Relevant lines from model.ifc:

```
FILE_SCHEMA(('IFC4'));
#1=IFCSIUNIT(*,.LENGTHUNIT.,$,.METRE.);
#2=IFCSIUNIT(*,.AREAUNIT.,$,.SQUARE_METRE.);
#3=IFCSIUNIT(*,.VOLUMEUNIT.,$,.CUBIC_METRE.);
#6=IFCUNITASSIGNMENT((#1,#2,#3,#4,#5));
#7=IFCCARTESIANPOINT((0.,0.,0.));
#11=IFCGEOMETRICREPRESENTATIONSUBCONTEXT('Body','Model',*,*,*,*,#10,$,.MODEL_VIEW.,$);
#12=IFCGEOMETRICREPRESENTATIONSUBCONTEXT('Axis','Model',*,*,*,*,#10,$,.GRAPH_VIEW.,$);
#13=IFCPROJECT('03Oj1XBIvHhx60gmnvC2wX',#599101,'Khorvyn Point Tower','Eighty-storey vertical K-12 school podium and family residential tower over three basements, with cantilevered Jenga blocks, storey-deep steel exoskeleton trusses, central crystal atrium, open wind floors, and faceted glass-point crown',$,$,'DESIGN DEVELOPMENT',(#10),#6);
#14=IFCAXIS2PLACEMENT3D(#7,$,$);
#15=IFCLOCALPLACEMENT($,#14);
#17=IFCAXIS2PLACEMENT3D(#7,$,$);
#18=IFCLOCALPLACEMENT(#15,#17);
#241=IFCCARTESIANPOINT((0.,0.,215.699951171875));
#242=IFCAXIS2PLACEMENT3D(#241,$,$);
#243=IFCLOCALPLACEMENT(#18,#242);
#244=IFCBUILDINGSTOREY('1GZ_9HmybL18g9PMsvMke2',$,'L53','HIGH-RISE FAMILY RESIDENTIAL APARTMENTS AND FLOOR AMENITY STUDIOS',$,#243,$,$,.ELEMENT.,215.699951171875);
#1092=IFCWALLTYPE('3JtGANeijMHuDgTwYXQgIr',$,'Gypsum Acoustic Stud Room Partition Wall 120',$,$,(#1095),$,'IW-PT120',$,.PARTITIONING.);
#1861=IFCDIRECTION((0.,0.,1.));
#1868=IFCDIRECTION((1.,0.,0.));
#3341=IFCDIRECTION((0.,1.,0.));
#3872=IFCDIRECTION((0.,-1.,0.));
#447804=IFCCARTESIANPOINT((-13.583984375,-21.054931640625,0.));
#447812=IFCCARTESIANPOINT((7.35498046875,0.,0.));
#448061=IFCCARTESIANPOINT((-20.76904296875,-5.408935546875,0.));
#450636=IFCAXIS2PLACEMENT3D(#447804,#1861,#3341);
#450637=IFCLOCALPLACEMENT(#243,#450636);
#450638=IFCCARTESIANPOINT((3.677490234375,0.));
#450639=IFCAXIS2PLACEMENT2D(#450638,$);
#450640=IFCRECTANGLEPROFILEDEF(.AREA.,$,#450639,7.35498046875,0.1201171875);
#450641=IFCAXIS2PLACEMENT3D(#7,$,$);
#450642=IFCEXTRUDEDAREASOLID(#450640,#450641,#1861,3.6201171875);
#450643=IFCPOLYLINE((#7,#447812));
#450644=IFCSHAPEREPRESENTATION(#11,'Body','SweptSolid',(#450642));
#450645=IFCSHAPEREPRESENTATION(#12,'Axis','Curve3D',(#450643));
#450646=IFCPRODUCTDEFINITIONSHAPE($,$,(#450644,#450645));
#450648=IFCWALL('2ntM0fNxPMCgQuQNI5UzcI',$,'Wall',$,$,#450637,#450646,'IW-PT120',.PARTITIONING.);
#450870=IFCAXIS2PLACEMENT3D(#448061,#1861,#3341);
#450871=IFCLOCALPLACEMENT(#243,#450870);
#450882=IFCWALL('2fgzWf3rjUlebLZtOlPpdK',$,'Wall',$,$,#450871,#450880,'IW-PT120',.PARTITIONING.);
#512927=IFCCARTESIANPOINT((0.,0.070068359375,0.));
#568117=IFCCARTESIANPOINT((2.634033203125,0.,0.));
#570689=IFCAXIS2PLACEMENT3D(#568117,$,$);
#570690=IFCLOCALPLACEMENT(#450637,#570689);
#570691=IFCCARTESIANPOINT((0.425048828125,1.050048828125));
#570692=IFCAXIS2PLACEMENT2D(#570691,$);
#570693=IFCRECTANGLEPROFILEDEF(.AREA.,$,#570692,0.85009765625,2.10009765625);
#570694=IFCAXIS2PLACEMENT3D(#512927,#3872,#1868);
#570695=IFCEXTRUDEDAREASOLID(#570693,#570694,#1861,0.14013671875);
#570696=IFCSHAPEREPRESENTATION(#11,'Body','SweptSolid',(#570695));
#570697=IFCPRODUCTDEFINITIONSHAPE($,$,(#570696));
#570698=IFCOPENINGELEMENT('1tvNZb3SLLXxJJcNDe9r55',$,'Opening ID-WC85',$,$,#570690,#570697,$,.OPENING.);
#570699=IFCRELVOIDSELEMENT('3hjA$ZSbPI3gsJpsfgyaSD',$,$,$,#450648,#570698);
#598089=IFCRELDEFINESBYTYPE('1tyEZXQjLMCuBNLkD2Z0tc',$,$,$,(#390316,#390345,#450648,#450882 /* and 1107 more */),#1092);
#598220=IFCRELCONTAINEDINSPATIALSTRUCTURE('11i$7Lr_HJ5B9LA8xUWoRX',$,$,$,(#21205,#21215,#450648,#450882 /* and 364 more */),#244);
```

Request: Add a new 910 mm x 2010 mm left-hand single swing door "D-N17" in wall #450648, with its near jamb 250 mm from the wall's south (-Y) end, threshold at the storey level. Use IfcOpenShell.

```python
import numpy as np
import ifcopenshell
import ifcopenshell.api.feature
import ifcopenshell.api.geometry
import ifcopenshell.api.root
import ifcopenshell.api.spatial
import ifcopenshell.geom
import ifcopenshell.util.element
import ifcopenshell.util.placement
import ifcopenshell.util.representation
import ifcopenshell.util.shape
import ifcopenshell.util.unit

model = ifcopenshell.open("model.ifc")
unit_scale = ifcopenshell.util.unit.calculate_unit_scale(model)
settings = ifcopenshell.geom.settings()


def volume(element):
    """Net volume in cubic metres, openings subtracted."""
    shape = ifcopenshell.geom.create_shape(settings, element)
    return ifcopenshell.util.shape.get_volume(shape.geometry)


wall = model.by_guid("2ntM0fNxPMCgQuQNI5UzcI")
storey = ifcopenshell.util.element.get_container(wall, ifc_class="IfcBuildingStorey")
context = ifcopenshell.util.representation.get_context(model, "Model", "Body", "MODEL_VIEW")
before = volume(wall)

width, height, from_end, sill = 0.91, 2.01, 0.25, 0.0  # metres

# The wall runs along its own X axis, and the end named is its -X end.
wall_shape = ifcopenshell.geom.create_shape(settings, wall)
x, y, z = ifcopenshell.util.shape.get_vertices(wall_shape.geometry).T
start = x.min() + from_end
face, thickness = float(y.min()), float(y.max() - y.min())
wall_matrix = ifcopenshell.util.placement.get_local_placement(wall.ObjectPlacement)
level = ifcopenshell.util.placement.get_local_placement(storey.ObjectPlacement)[2, 3]


def in_wall(x, y):
    """Placement at x, y metres in the wall's axes, at sill height."""
    matrix = wall_matrix.copy()
    matrix[:, 3] = wall_matrix @ np.array([x / unit_scale, y / unit_scale, 0.0, 1.0])
    matrix[2, 3] = level + sill / unit_scale
    return matrix


# Opening: a box that overshoots both wall faces by 50 mm.
opening = ifcopenshell.api.root.create_entity(model, ifc_class="IfcOpeningElement", predefined_type="OPENING")
box = ifcopenshell.api.geometry.add_wall_representation(
    model, context=context, length=width, height=height, thickness=thickness + 0.1
)
ifcopenshell.api.geometry.assign_representation(model, product=opening, representation=box)
ifcopenshell.api.geometry.edit_object_placement(model, product=opening, matrix=in_wall(start, face - 0.05), is_si=False)
ifcopenshell.api.feature.add_feature(model, feature=opening, element=wall)

door = ifcopenshell.api.root.create_entity(model, ifc_class="IfcDoor", name="D-N17", predefined_type="DOOR")
door.OverallWidth, door.OverallHeight = width / unit_scale, height / unit_scale
door.OperationType = "SINGLE_SWING_LEFT"
body = ifcopenshell.api.geometry.add_door_representation(
    model,
    context=context,
    overall_width=door.OverallWidth,
    overall_height=door.OverallHeight,
    operation_type="SINGLE_SWING_LEFT",
    lining_properties={"LiningDepth": thickness / unit_scale, "ThresholdDepth": thickness / unit_scale},
)
ifcopenshell.api.geometry.assign_representation(model, product=door, representation=body)
ifcopenshell.api.spatial.assign_container(model, products=[door], relating_structure=storey)
ifcopenshell.api.feature.add_filling(model, opening=opening, element=door)

# The lining spans the wall, so the door starts at the wall face.
ifcopenshell.api.geometry.edit_object_placement(model, product=door, matrix=in_wall(start, face), is_si=False)

after = volume(wall)

print(f"wall volume {before:.3f} -> {after:.3f} m3")

model.write("model_rev.ifc")
```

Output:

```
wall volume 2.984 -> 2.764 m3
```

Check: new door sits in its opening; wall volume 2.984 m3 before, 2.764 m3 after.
